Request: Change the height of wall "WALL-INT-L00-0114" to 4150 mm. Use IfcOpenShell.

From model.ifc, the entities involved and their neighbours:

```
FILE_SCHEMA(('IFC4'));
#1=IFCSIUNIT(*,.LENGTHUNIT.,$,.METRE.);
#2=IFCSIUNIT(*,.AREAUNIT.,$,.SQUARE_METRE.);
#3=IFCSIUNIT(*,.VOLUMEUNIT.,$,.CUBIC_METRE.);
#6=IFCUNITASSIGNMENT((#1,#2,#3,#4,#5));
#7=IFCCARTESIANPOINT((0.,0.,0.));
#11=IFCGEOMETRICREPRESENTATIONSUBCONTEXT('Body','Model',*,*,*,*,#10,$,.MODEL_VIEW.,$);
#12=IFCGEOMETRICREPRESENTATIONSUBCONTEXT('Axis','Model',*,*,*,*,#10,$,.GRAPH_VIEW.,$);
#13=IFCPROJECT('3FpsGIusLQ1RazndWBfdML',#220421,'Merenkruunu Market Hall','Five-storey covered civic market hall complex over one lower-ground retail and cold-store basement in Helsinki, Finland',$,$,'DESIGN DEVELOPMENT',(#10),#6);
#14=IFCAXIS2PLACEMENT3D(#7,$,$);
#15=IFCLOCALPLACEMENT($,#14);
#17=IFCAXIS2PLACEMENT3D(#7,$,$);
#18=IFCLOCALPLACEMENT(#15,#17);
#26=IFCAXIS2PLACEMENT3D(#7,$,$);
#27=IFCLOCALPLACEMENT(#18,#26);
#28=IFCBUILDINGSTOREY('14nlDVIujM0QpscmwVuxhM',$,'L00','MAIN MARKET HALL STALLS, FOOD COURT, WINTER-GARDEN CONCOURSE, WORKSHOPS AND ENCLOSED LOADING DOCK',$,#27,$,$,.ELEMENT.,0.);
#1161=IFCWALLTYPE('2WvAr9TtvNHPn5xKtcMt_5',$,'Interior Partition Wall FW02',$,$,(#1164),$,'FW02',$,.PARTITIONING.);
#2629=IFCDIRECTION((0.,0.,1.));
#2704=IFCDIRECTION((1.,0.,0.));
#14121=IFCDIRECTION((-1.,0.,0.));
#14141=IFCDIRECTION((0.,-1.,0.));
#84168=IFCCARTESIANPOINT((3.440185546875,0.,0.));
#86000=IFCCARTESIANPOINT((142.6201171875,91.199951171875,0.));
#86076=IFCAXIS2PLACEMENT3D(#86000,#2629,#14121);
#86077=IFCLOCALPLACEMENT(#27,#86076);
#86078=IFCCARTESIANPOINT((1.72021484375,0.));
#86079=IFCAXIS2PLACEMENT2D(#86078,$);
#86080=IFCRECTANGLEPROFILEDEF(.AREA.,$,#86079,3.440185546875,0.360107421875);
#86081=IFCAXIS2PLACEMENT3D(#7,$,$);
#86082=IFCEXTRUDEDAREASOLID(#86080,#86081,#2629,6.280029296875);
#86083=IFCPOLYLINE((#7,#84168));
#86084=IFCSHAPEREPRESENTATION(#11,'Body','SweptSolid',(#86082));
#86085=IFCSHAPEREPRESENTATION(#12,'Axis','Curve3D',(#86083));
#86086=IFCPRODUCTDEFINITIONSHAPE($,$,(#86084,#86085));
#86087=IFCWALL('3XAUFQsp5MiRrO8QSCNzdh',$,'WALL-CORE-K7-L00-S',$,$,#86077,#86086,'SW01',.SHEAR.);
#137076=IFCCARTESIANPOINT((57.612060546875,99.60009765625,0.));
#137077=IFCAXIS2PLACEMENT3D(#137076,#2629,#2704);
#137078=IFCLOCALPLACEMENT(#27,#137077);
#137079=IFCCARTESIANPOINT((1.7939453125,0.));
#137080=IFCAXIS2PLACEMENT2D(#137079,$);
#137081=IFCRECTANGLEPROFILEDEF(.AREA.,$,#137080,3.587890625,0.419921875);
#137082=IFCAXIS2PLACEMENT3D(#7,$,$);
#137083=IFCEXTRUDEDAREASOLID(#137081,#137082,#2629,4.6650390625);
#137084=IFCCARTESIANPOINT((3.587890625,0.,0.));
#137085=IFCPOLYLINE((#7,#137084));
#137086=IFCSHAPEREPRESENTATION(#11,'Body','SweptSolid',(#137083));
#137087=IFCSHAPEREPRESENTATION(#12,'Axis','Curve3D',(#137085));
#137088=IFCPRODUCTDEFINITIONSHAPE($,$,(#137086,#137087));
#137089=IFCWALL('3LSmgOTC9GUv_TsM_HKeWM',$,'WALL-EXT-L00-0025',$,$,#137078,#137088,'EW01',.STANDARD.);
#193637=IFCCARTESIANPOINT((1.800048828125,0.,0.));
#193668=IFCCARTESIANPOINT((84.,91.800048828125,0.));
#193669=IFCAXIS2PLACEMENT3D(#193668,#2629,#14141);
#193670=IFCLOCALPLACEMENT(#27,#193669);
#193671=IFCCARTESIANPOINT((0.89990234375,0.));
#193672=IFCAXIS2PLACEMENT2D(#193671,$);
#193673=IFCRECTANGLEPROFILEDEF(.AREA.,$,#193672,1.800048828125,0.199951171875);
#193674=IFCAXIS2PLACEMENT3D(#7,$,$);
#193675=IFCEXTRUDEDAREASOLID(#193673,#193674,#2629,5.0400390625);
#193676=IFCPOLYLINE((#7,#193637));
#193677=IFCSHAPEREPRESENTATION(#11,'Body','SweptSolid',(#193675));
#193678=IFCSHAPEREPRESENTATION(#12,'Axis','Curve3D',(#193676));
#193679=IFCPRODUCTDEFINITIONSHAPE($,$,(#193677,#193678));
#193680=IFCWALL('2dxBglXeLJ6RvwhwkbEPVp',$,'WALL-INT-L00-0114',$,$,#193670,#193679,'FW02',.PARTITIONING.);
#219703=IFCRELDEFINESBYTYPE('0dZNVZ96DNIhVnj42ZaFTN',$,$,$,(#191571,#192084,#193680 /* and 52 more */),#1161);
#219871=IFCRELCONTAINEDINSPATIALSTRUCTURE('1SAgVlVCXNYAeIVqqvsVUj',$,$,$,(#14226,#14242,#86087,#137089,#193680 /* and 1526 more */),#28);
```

```python
import ifcopenshell
import ifcopenshell.geom
import ifcopenshell.util.representation
import ifcopenshell.util.shape
import ifcopenshell.util.unit

model = ifcopenshell.open("model.ifc")
unit_scale = ifcopenshell.util.unit.calculate_unit_scale(model)
settings = ifcopenshell.geom.settings()


def volume(element):
    """Net volume in cubic metres, openings subtracted."""
    shape = ifcopenshell.geom.create_shape(settings, element)
    return ifcopenshell.util.shape.get_volume(shape.geometry)


wall = model.by_guid("2dxBglXeLJ6RvwhwkbEPVp")
before = volume(wall)

body = ifcopenshell.util.representation.get_representation(wall, "Model", "Body")
solid = body.Items[0]
old_height = solid.Depth
solid.Depth = 4.15 / unit_scale
after = volume(wall)

print(f"height {old_height:g} -> {solid.Depth:g}, volume {before:.3f} -> {after:.3f} m3")

model.write("model-out.ifc")
```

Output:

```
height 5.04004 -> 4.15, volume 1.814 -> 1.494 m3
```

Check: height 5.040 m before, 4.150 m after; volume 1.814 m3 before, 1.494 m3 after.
